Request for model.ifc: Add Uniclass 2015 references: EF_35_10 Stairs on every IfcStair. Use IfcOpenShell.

First a look at what the model holds.

```python
import ifcopenshell

model = ifcopenshell.open("model.ifc")
print(model.schema)
print("classifications:", [c.Name for c in model.by_type("IfcClassification")])
for ifc_class in ("IfcDoor", "IfcRoof", "IfcStair", "IfcWall", "IfcWindow"):
    print(ifc_class, len(model.by_type(ifc_class)))
```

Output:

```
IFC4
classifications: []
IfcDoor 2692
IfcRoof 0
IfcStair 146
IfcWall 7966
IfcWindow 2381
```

```python
import ifcopenshell
import ifcopenshell.api.classification

model = ifcopenshell.open("model.ifc")

system = ifcopenshell.api.classification.add_classification(model, classification="Uniclass 2015")

codes = {
    "IfcStair": ("EF_35_10", "Stairs"),
}
for ifc_class, (code, name) in codes.items():
    products = model.by_type(ifc_class)
    ifcopenshell.api.classification.add_reference(
        model, products=products, classification=system, identification=code, name=name
    )
    print(code, len(products))

model.write("model_updated.ifc")
```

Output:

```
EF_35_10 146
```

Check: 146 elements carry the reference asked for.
